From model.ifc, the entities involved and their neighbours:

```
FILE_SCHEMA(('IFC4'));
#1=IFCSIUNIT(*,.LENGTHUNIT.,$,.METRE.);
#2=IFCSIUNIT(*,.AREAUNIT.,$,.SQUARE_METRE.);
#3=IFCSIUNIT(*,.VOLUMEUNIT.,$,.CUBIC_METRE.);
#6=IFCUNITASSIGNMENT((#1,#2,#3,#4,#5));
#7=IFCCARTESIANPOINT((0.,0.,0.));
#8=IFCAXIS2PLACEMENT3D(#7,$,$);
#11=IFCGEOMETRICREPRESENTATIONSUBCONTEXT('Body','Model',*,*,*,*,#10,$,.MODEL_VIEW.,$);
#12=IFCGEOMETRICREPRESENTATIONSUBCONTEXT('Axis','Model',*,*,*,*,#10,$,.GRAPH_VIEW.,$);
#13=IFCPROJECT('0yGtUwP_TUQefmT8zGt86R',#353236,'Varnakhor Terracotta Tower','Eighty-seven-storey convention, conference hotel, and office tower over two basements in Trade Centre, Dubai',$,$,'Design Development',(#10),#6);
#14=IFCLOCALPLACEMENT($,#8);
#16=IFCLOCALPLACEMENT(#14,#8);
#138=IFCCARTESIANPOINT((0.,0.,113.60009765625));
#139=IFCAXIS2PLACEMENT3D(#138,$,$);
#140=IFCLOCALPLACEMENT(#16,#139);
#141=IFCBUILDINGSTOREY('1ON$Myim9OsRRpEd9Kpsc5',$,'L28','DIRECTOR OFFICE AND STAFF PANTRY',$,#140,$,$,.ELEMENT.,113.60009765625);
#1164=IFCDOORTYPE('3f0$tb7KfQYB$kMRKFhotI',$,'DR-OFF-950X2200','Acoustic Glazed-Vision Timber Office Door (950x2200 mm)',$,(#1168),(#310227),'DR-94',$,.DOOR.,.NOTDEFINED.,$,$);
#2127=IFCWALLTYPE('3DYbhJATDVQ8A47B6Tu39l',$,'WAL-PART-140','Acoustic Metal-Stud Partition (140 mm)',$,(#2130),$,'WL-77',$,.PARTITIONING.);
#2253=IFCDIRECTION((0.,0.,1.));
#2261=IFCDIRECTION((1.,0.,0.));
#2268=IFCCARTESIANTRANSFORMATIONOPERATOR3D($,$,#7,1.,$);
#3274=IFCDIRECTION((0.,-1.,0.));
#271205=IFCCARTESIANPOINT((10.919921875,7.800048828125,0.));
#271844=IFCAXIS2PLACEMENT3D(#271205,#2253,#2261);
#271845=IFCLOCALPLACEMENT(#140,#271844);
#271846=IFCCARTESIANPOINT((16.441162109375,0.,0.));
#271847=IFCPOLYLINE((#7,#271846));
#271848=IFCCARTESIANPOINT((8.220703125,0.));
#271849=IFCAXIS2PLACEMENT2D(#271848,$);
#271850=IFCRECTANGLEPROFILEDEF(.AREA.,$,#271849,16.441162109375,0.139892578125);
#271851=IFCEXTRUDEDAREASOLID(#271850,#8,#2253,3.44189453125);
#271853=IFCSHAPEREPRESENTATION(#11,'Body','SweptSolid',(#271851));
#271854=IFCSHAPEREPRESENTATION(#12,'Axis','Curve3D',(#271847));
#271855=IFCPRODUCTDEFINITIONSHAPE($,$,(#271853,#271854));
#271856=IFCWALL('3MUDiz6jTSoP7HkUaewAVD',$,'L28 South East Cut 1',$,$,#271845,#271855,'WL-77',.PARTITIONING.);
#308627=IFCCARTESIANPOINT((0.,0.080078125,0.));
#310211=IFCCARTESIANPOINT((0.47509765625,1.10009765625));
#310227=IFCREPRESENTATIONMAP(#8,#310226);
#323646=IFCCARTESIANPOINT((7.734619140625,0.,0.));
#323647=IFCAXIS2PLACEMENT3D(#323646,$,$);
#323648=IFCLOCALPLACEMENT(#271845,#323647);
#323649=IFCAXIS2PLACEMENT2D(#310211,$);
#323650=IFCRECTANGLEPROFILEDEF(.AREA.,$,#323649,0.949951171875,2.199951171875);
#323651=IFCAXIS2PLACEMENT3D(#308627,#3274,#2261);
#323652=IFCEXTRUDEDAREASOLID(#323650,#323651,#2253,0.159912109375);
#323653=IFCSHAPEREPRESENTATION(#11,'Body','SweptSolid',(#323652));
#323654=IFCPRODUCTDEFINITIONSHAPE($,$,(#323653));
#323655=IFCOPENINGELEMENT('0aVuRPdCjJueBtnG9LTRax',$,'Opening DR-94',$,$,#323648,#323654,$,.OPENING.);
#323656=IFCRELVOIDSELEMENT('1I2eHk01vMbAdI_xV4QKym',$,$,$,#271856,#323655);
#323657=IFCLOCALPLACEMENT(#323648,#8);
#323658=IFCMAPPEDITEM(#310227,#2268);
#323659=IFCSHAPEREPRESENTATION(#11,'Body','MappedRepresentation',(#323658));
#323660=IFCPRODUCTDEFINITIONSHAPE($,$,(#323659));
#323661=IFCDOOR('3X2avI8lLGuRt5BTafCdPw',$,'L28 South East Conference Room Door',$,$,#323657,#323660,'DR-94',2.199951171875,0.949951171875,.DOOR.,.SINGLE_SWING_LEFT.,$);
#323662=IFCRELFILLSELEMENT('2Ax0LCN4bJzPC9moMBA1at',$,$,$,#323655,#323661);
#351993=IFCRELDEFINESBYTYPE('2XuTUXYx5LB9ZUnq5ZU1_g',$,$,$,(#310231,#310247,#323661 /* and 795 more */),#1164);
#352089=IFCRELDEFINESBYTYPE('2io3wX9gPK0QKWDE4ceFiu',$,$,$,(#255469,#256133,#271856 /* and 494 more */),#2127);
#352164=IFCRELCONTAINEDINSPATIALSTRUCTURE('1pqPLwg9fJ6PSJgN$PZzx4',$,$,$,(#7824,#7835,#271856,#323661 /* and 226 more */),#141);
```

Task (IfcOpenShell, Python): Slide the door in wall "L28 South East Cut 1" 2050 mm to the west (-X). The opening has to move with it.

```python
import ifcopenshell
import ifcopenshell.api.geometry
import ifcopenshell.util.placement

model = ifcopenshell.open("model.ifc")

door = model.by_guid("3X2avI8lLGuRt5BTafCdPw")
opening = door.FillsVoids[0].RelatingOpeningElement
wall = opening.VoidsElements[0].RelatingBuildingElement

wall_matrix = ifcopenshell.util.placement.get_local_placement(wall.ObjectPlacement)
shift = wall_matrix[:3, 0] * -2.05
before = ifcopenshell.util.placement.get_local_placement(door.ObjectPlacement)[:3, 3].copy()

# The door is placed relative to its opening, so it follows when the opening moves.
matrix = ifcopenshell.util.placement.get_local_placement(opening.ObjectPlacement)
matrix[:3, 3] += shift
ifcopenshell.api.geometry.edit_object_placement(
    model, product=opening, matrix=matrix, is_si=False, should_transform_children=True
)

after = ifcopenshell.util.placement.get_local_placement(door.ObjectPlacement)[:3, 3]
print("door moved by", (after - before).round(3) + 0.0)

model.write("model_rev.ifc")
```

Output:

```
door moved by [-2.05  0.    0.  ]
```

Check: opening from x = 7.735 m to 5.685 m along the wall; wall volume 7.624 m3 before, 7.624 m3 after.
